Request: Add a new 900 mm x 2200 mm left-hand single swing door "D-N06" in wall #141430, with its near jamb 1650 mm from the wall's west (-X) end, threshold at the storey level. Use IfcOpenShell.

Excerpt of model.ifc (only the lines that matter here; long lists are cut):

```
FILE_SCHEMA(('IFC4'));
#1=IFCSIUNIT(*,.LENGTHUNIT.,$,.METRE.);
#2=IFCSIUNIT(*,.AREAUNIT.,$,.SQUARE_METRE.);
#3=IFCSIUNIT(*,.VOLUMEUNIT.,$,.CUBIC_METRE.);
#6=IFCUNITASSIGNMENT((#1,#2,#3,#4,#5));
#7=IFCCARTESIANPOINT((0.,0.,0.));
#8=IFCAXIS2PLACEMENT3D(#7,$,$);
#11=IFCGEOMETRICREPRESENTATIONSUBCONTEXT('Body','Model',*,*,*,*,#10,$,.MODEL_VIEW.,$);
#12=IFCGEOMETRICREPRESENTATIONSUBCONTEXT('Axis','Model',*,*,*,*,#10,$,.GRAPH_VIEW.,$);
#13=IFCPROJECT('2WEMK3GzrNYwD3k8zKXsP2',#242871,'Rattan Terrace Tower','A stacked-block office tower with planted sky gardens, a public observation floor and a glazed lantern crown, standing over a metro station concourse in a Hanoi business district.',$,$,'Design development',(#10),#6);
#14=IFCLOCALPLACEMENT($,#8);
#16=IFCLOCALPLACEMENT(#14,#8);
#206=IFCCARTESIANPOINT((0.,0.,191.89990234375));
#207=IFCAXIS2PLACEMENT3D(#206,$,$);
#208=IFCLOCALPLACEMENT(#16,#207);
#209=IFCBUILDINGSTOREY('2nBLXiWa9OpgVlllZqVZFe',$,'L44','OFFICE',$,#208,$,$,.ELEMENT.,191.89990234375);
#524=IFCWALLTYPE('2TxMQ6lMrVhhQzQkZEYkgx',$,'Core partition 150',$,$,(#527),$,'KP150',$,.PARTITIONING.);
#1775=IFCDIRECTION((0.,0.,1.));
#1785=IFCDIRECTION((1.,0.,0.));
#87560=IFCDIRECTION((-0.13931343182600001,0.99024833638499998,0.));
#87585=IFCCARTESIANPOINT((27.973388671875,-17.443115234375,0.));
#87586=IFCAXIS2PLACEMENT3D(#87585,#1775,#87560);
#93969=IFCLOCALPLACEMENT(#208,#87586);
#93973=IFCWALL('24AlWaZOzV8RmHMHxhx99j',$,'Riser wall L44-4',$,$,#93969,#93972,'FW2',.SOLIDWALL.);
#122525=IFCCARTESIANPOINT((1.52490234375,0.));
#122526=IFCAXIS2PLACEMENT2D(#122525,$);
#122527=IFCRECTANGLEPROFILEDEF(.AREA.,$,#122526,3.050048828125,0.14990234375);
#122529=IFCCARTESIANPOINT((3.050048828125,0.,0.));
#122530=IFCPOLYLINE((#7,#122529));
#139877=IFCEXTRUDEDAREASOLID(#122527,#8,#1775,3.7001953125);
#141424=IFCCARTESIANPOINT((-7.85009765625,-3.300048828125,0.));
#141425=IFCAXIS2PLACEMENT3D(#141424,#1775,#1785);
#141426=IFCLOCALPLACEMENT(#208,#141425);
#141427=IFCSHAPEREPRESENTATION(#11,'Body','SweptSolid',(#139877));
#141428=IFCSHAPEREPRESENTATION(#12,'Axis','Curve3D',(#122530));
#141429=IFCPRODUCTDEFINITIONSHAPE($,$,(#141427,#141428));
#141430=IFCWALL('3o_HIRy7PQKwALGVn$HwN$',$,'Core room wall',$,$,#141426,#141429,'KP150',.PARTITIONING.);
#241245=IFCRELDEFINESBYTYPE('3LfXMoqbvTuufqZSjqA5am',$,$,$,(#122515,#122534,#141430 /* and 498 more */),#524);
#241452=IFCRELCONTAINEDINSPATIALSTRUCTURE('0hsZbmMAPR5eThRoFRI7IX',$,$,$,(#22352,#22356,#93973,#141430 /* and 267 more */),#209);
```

```python
import numpy as np
import ifcopenshell
import ifcopenshell.api.feature
import ifcopenshell.api.geometry
import ifcopenshell.api.root
import ifcopenshell.api.spatial
import ifcopenshell.geom
import ifcopenshell.util.element
import ifcopenshell.util.placement
import ifcopenshell.util.representation
import ifcopenshell.util.shape
import ifcopenshell.util.unit

model = ifcopenshell.open("model.ifc")
unit_scale = ifcopenshell.util.unit.calculate_unit_scale(model)
settings = ifcopenshell.geom.settings()


def volume(element):
    """Net volume in cubic metres, openings subtracted."""
    shape = ifcopenshell.geom.create_shape(settings, element)
    return ifcopenshell.util.shape.get_volume(shape.geometry)


wall = model.by_guid("3o_HIRy7PQKwALGVn$HwN$")
storey = ifcopenshell.util.element.get_container(wall, ifc_class="IfcBuildingStorey")
context = ifcopenshell.util.representation.get_context(model, "Model", "Body", "MODEL_VIEW")
before = volume(wall)

width, height, from_end, sill = 0.9, 2.2, 1.65, 0.0  # metres

# The wall runs along its own X axis, and the end named is its -X end.
wall_shape = ifcopenshell.geom.create_shape(settings, wall)
x, y, z = ifcopenshell.util.shape.get_vertices(wall_shape.geometry).T
start = x.min() + from_end
face, thickness = float(y.min()), float(y.max() - y.min())
wall_matrix = ifcopenshell.util.placement.get_local_placement(wall.ObjectPlacement)
level = ifcopenshell.util.placement.get_local_placement(storey.ObjectPlacement)[2, 3]


def in_wall(x, y):
    """Placement at x, y metres in the wall's axes, at sill height."""
    matrix = wall_matrix.copy()
    matrix[:, 3] = wall_matrix @ np.array([x / unit_scale, y / unit_scale, 0.0, 1.0])
    matrix[2, 3] = level + sill / unit_scale
    return matrix


# Opening: a box that overshoots both wall faces by 50 mm.
opening = ifcopenshell.api.root.create_entity(model, ifc_class="IfcOpeningElement", predefined_type="OPENING")
box = ifcopenshell.api.geometry.add_wall_representation(
    model, context=context, length=width, height=height, thickness=thickness + 0.1
)
ifcopenshell.api.geometry.assign_representation(model, product=opening, representation=box)
ifcopenshell.api.geometry.edit_object_placement(model, product=opening, matrix=in_wall(start, face - 0.05), is_si=False)
ifcopenshell.api.feature.add_feature(model, feature=opening, element=wall)

door = ifcopenshell.api.root.create_entity(model, ifc_class="IfcDoor", name="D-N06", predefined_type="DOOR")
door.OverallWidth, door.OverallHeight = width / unit_scale, height / unit_scale
door.OperationType = "SINGLE_SWING_LEFT"
body = ifcopenshell.api.geometry.add_door_representation(
    model,
    context=context,
    overall_width=door.OverallWidth,
    overall_height=door.OverallHeight,
    operation_type="SINGLE_SWING_LEFT",
    lining_properties={"LiningDepth": thickness / unit_scale, "ThresholdDepth": thickness / unit_scale},
)
ifcopenshell.api.geometry.assign_representation(model, product=door, representation=body)
ifcopenshell.api.spatial.assign_container(model, products=[door], relating_structure=storey)
ifcopenshell.api.feature.add_filling(model, opening=opening, element=door)

# The lining spans the wall, so the door starts at the wall face.
ifcopenshell.api.geometry.edit_object_placement(model, product=door, matrix=in_wall(start, face), is_si=False)

after = volume(wall)

print(f"wall volume {before:.3f} -> {after:.3f} m3")

model.write("model_updated.ifc")
```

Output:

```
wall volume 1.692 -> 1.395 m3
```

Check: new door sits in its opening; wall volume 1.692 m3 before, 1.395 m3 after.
